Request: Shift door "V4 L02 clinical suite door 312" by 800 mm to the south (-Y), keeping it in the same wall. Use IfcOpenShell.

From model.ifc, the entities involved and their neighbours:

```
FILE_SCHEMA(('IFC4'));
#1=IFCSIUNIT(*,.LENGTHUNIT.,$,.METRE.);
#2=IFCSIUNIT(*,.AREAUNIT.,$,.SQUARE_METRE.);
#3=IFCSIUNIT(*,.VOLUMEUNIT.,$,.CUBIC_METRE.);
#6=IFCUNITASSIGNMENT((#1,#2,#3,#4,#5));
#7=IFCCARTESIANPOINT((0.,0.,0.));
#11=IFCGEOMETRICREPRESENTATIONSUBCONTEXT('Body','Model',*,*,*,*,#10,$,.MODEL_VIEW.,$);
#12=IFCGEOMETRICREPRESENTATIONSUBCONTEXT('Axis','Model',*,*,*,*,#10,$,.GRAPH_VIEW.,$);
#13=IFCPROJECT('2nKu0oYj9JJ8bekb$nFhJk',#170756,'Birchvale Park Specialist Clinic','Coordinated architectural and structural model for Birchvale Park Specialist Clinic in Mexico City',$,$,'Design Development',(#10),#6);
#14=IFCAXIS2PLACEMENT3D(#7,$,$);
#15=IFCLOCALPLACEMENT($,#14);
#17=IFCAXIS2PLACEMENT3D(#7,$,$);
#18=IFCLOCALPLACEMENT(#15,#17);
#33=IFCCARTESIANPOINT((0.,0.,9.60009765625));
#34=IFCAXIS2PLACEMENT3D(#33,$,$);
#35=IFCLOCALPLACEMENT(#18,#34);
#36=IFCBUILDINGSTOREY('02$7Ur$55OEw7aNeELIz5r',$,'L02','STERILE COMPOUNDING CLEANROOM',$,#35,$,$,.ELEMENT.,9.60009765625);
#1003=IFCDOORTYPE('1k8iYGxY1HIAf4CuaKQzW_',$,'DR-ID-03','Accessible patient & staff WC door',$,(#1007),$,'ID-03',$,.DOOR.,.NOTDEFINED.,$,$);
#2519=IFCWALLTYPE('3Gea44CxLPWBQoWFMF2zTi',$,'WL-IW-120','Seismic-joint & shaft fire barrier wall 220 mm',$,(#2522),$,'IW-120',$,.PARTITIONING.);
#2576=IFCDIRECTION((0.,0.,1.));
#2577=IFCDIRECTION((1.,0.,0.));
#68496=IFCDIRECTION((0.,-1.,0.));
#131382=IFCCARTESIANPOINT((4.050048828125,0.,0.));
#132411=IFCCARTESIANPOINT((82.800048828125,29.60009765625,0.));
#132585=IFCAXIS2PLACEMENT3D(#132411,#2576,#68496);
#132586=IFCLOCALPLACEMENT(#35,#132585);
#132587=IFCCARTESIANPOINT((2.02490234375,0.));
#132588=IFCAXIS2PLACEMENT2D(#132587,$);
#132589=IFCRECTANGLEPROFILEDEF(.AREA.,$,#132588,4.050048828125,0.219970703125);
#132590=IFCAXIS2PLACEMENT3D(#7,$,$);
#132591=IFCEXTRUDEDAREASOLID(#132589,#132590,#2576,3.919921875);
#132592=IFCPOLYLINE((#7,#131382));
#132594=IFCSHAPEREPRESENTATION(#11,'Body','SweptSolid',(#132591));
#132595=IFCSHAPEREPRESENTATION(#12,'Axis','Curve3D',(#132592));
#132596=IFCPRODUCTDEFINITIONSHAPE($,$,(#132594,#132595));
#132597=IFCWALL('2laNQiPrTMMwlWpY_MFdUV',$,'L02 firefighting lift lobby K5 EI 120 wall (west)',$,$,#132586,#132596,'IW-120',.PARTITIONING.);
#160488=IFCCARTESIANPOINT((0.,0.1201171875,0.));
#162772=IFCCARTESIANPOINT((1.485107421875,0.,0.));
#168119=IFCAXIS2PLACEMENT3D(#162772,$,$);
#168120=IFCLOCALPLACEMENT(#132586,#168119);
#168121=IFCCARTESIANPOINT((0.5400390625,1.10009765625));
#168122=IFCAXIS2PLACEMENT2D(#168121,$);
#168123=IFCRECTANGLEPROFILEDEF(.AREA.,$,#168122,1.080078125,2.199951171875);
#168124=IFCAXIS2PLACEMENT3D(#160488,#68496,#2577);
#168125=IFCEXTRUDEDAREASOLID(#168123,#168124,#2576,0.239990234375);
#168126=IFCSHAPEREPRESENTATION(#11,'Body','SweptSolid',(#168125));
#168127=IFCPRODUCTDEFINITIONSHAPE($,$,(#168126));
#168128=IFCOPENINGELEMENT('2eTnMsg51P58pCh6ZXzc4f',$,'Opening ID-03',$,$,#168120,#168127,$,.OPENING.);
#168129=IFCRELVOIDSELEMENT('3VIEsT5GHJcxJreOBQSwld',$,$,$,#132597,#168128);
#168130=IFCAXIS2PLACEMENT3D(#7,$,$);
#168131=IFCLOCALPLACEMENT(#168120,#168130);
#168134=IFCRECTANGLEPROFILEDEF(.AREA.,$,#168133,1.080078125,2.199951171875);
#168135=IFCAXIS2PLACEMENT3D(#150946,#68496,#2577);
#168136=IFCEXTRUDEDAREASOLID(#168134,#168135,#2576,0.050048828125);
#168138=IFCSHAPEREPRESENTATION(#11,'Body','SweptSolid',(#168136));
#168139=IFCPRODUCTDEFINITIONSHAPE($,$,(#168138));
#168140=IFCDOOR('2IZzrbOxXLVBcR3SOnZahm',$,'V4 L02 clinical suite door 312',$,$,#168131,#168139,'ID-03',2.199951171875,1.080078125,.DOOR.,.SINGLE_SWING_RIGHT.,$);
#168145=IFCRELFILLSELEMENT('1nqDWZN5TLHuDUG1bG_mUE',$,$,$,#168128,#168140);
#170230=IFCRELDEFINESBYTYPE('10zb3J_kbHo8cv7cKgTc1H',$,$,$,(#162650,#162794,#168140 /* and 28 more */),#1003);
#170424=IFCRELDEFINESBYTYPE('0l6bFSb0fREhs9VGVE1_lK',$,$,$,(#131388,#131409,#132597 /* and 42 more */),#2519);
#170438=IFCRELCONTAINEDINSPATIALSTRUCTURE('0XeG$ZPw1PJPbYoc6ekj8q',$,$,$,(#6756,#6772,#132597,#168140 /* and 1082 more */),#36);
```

```python
import ifcopenshell
import ifcopenshell.api.geometry
import ifcopenshell.util.placement

model = ifcopenshell.open("model.ifc")

door = model.by_guid("2IZzrbOxXLVBcR3SOnZahm")
opening = door.FillsVoids[0].RelatingOpeningElement
wall = opening.VoidsElements[0].RelatingBuildingElement

wall_matrix = ifcopenshell.util.placement.get_local_placement(wall.ObjectPlacement)
shift = wall_matrix[:3, 0] * 0.8
before = ifcopenshell.util.placement.get_local_placement(door.ObjectPlacement)[:3, 3].copy()

# The door is placed relative to its opening, so it follows when the opening moves.
matrix = ifcopenshell.util.placement.get_local_placement(opening.ObjectPlacement)
matrix[:3, 3] += shift
ifcopenshell.api.geometry.edit_object_placement(
    model, product=opening, matrix=matrix, is_si=False, should_transform_children=True
)

after = ifcopenshell.util.placement.get_local_placement(door.ObjectPlacement)[:3, 3]
print("door moved by", (after - before).round(3) + 0.0)

model.write("model_rev.ifc")
```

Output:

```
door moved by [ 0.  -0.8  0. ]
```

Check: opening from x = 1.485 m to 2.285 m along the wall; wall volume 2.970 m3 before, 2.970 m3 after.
